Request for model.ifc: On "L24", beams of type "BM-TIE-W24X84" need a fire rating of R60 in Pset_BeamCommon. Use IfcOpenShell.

First a look at what the model holds.

```python
import ifcopenshell
import ifcopenshell.util.element

model = ifcopenshell.open("model.ifc")
print(model.schema)
storey = next(s for s in model.by_type("IfcBuildingStorey") if s.Name == "L24")
beams = [e for e in ifcopenshell.util.element.get_decomposition(storey) if e.is_a("IfcBeam")]
seen = {}
for e in beams:
    element_type = ifcopenshell.util.element.get_type(e)
    key = (element_type.Name if element_type != e and element_type else None, ifcopenshell.util.element.get_pset(e, "Pset_BeamCommon", "FireRating"))
    seen[key] = seen.get(key, 0) + 1
for (name, value), count in sorted(seen.items(), key=str):
    print(count, "x", name, "|", value)
```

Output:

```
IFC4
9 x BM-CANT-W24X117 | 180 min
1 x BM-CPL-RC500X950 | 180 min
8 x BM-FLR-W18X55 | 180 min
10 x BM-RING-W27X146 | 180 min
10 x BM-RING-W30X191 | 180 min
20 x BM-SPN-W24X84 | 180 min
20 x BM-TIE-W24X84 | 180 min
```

```python
import ifcopenshell
import ifcopenshell.api.pset
import ifcopenshell.util.element

model = ifcopenshell.open("model.ifc")

storey = next(s for s in model.by_type("IfcBuildingStorey") if s.Name == "L24")
beams = [e for e in ifcopenshell.util.element.get_decomposition(storey) if e.is_a("IfcBeam")]

count = 0
for e in beams:
    element_type = ifcopenshell.util.element.get_type(e)
    if element_type in (None, e) or element_type.Name != "BM-TIE-W24X84":
        continue
    # add_pset returns the element's existing set when there is one.
    pset = ifcopenshell.api.pset.add_pset(model, product=e, name="Pset_BeamCommon")
    ifcopenshell.api.pset.edit_pset(model, pset=pset, properties={"FireRating": "R60"})
    count += 1

print(count, "beams updated")

model.write("model_rev.ifc")
```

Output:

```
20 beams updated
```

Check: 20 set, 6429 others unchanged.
